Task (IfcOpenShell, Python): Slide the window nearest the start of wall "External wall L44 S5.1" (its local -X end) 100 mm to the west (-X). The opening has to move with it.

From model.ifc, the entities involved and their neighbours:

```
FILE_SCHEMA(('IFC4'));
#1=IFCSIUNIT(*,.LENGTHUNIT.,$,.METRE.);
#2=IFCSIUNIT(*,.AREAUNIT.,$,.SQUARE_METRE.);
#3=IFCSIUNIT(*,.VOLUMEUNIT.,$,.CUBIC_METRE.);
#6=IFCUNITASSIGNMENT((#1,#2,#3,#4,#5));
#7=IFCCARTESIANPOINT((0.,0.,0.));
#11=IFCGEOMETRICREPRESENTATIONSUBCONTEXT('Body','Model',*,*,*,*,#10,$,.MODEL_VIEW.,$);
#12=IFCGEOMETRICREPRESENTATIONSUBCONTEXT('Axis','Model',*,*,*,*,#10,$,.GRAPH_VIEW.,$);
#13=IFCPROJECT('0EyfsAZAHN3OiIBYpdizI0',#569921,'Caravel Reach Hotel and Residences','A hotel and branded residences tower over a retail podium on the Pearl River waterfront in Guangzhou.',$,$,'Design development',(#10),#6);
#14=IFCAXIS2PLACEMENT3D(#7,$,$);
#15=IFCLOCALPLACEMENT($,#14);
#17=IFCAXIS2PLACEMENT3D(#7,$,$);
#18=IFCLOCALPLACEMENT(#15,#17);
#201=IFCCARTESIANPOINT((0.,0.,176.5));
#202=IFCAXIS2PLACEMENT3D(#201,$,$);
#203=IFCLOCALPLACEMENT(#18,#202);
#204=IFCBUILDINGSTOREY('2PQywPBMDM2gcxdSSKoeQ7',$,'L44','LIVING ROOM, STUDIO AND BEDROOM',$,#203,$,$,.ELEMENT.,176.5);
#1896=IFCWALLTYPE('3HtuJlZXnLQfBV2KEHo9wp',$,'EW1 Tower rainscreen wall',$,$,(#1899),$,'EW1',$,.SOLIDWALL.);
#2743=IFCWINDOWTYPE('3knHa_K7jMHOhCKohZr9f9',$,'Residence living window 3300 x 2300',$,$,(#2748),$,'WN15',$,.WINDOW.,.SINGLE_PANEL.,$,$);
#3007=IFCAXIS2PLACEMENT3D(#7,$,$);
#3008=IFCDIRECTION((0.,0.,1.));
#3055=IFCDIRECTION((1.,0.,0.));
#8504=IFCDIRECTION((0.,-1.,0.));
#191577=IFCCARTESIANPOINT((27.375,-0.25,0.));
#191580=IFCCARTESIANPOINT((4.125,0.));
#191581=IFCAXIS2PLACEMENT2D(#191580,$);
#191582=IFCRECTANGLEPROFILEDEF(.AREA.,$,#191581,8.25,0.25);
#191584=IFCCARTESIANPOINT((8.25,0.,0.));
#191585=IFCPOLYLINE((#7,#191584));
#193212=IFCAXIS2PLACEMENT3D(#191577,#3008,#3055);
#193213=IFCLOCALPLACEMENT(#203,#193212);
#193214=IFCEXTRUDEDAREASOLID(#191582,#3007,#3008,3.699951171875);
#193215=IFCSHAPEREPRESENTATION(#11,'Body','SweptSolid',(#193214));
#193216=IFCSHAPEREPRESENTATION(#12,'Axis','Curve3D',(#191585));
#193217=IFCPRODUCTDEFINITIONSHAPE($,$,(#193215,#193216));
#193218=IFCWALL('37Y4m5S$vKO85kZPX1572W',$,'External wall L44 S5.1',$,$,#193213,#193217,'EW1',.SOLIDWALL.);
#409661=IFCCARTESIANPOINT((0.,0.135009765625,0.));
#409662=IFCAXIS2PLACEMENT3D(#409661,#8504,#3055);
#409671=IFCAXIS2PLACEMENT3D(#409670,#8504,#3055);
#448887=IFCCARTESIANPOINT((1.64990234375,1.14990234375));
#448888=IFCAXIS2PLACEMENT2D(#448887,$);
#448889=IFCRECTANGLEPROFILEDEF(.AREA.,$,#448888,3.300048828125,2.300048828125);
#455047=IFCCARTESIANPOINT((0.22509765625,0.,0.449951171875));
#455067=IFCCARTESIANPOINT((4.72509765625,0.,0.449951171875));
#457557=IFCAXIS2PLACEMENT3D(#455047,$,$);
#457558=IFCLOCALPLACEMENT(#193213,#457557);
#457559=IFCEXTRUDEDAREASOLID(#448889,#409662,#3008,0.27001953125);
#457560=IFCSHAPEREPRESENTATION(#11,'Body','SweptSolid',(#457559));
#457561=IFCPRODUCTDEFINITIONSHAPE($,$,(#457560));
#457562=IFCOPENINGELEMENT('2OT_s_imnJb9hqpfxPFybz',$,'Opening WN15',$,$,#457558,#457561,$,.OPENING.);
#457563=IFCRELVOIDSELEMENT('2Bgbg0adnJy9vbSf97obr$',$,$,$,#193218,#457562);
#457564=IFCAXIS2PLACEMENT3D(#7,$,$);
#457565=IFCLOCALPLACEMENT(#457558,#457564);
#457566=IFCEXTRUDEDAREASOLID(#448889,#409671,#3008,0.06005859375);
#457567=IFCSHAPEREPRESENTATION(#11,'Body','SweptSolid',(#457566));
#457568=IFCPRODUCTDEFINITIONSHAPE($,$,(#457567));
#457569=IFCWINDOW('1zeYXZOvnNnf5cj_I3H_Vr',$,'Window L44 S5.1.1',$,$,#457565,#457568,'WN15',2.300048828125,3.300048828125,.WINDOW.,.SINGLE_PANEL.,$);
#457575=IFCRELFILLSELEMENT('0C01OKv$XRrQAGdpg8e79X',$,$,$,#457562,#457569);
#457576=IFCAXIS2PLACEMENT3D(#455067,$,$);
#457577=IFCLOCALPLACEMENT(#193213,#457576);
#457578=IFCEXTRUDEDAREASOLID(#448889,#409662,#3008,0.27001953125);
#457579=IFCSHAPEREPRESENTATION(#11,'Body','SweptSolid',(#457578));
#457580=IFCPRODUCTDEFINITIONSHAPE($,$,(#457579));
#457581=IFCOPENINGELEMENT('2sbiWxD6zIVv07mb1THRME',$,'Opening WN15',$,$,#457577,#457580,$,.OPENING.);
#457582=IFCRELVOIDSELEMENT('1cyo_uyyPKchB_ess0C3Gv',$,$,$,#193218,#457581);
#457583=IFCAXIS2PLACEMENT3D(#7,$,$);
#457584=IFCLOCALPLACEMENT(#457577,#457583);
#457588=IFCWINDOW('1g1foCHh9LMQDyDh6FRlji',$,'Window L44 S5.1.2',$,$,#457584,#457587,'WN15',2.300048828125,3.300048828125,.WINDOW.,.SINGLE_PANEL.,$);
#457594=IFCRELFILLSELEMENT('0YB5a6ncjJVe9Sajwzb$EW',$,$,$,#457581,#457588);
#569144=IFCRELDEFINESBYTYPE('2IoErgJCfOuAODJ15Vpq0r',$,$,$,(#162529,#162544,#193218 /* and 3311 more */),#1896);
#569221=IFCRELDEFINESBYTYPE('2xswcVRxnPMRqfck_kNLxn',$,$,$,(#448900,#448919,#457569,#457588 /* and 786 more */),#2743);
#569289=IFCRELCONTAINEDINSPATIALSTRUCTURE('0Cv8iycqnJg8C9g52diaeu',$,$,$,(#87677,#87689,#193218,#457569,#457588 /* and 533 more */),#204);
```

```python
import ifcopenshell
import ifcopenshell.api.geometry
import ifcopenshell.util.placement
import ifcopenshell.util.unit

model = ifcopenshell.open("model.ifc")
unit_scale = ifcopenshell.util.unit.calculate_unit_scale(model)

window = model.by_guid("1zeYXZOvnNnf5cj_I3H_Vr")
opening = window.FillsVoids[0].RelatingOpeningElement
wall = opening.VoidsElements[0].RelatingBuildingElement

wall_matrix = ifcopenshell.util.placement.get_local_placement(wall.ObjectPlacement)
shift = wall_matrix[:3, 0] * -0.1 / unit_scale
before = ifcopenshell.util.placement.get_local_placement(window.ObjectPlacement)[:3, 3].copy()

# The window is placed relative to its opening, so it follows when the opening moves.
matrix = ifcopenshell.util.placement.get_local_placement(opening.ObjectPlacement)
matrix[:3, 3] += shift
ifcopenshell.api.geometry.edit_object_placement(
    model, product=opening, matrix=matrix, is_si=False, should_transform_children=True
)

after = ifcopenshell.util.placement.get_local_placement(window.ObjectPlacement)[:3, 3]
print("window moved by", (after - before).round(3) + 0.0)

model.write("model_updated.ifc")
```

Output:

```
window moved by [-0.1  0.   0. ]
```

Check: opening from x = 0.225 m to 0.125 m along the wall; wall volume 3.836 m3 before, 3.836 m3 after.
